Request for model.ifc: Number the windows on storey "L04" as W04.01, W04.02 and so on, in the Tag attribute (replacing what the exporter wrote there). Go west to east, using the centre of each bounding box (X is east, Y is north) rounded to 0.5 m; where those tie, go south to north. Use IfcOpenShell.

First a look at what the model holds.

```python
import ifcopenshell
import ifcopenshell.util.element
import ifcopenshell.util.placement

model = ifcopenshell.open("model.ifc")
print(model.schema)
storey = next(s for s in model.by_type("IfcBuildingStorey") if s.Name == "L04")
windows = [e for e in ifcopenshell.util.element.get_decomposition(storey) if e.is_a("IfcWindow")]
for e in sorted(windows, key=lambda e: e.id()):
    origin = ifcopenshell.util.placement.get_local_placement(e.ObjectPlacement)[:3, 3]
    print(e.id(), e.Tag, e.Name, origin.round(2) + 0.0, sep=" | ")
```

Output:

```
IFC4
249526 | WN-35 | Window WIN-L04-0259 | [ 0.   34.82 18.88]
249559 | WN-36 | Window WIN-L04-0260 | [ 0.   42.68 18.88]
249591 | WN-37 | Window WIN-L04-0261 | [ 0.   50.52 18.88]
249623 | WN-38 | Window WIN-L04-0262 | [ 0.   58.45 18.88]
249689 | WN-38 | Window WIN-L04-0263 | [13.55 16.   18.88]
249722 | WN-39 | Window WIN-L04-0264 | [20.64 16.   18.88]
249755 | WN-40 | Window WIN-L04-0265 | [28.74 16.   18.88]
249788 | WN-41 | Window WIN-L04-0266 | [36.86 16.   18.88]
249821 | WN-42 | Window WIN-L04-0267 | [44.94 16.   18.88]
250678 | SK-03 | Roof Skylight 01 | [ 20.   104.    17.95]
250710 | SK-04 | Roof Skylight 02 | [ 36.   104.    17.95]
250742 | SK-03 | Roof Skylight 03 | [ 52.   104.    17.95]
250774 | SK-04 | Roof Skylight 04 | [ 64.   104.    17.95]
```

```python
import ifcopenshell
import ifcopenshell.geom
import ifcopenshell.util.element
import ifcopenshell.util.shape

model = ifcopenshell.open("model.ifc")
settings = ifcopenshell.geom.settings()
settings.set("use-world-coords", True)


def centre(element):
    shape = ifcopenshell.geom.create_shape(settings, element)
    return ifcopenshell.util.shape.get_bbox_centroid(shape.geometry)


storey = next(s for s in model.by_type("IfcBuildingStorey") if s.Name == "L04")
windows = [e for e in ifcopenshell.util.element.get_decomposition(storey) if e.is_a("IfcWindow")]

# Insertion points can sit at a corner or the storey origin, so sort by the geometry (in metres).
centres = {e: centre(e) for e in windows}
windows.sort(key=lambda e: (round(centres[e][0] / 0.5), centres[e][1]))

for i, e in enumerate(windows, start=1):
    number = f"W04.{i:02d}"
    e.Tag = number
    print(e.id(), number)

model.write("model_updated.ifc")
```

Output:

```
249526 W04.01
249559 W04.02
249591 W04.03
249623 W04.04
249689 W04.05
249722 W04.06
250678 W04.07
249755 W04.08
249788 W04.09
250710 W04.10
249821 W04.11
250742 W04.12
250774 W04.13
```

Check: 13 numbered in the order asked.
